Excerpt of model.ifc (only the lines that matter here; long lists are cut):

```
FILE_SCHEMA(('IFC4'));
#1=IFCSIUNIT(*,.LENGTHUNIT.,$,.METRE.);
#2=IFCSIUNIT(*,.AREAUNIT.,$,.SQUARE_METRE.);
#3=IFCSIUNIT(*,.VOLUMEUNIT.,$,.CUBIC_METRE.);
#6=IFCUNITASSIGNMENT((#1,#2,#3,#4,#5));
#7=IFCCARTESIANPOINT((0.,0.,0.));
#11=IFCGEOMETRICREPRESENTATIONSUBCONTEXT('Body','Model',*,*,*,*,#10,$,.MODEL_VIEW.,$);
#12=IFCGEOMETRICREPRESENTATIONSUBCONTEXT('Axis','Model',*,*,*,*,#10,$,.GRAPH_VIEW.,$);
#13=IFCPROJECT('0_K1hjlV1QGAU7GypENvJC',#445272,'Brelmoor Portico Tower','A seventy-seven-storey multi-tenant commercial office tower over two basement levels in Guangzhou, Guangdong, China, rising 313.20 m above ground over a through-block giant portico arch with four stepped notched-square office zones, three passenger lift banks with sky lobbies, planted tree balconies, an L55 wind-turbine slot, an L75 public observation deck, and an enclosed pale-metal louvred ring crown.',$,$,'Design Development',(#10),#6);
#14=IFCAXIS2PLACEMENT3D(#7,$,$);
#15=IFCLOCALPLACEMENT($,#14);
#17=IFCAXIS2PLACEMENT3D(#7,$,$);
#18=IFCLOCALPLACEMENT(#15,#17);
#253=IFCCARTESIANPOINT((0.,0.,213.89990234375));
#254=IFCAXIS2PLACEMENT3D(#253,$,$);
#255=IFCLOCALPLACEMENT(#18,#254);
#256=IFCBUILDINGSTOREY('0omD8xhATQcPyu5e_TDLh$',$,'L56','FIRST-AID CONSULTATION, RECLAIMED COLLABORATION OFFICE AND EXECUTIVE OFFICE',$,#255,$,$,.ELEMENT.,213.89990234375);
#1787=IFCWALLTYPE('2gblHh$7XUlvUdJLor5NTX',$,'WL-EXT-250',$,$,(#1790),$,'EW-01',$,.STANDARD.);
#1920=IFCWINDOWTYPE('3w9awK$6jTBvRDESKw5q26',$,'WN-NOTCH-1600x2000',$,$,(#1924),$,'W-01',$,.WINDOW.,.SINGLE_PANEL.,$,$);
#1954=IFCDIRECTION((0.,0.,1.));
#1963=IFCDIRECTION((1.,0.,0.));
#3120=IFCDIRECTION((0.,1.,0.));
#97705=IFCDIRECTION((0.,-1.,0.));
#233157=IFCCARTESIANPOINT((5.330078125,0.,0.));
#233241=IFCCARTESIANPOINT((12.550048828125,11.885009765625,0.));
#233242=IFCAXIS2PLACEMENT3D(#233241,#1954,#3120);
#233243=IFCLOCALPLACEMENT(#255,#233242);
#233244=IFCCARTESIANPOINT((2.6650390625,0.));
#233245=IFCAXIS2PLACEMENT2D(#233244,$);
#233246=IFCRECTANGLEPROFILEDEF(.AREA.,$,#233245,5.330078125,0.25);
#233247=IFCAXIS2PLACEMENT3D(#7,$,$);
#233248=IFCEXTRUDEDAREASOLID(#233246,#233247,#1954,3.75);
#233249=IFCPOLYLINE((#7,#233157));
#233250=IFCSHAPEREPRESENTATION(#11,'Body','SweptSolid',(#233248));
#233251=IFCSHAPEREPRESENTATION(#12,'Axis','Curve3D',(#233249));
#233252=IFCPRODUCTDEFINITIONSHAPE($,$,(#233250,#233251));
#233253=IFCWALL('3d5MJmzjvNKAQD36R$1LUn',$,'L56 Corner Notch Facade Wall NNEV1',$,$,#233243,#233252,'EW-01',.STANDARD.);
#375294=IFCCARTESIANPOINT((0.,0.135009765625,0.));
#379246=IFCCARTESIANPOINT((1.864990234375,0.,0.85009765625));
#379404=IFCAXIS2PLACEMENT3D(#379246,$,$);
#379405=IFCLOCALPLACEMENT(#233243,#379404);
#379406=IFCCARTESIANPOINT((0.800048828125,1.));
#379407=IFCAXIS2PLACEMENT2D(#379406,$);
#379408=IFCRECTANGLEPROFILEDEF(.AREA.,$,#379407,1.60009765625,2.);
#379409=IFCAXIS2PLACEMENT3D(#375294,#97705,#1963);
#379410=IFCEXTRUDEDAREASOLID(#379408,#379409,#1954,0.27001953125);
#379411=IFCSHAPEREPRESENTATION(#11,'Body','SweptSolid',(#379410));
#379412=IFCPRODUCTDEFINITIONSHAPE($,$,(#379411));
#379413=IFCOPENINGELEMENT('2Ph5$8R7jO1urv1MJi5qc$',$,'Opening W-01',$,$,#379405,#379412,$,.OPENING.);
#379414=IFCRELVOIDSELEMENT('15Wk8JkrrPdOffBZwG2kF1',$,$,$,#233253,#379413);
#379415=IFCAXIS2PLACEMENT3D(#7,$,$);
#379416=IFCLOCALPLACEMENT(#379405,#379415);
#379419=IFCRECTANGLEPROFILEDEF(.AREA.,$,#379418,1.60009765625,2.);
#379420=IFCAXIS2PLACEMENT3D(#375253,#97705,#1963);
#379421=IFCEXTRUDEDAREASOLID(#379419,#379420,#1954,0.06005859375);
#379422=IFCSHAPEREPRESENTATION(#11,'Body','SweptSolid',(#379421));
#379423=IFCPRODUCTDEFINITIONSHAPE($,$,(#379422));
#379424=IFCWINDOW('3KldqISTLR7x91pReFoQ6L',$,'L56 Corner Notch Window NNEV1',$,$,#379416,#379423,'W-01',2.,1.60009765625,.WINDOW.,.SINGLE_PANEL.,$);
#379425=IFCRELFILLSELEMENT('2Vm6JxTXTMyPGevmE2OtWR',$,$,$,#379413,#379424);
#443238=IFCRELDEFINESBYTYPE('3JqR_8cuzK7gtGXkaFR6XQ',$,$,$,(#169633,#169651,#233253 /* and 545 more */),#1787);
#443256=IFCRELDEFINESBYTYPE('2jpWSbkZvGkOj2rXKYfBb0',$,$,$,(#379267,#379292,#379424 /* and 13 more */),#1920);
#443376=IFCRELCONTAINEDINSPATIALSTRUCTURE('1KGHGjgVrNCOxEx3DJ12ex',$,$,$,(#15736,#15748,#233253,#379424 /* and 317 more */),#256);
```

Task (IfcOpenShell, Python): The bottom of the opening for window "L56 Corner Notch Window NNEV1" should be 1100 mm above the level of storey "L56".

```python
import numpy as np
import ifcopenshell
import ifcopenshell.api.geometry
import ifcopenshell.geom
import ifcopenshell.util.element
import ifcopenshell.util.placement
import ifcopenshell.util.shape
import ifcopenshell.util.unit

model = ifcopenshell.open("model.ifc")
unit_scale = ifcopenshell.util.unit.calculate_unit_scale(model)

window = model.by_id(379424)
opening = window.FillsVoids[0].RelatingOpeningElement
storey = ifcopenshell.util.element.get_container(window, ifc_class="IfcBuildingStorey")
level = ifcopenshell.util.placement.get_local_placement(storey.ObjectPlacement)[2, 3]

# The opening's origin need not be at the sill, so measure its lowest point.
shape = ifcopenshell.geom.create_shape(ifcopenshell.geom.settings(), opening)
bottom = ifcopenshell.util.shape.get_shape_bottom_elevation(shape, shape.geometry) / unit_scale
dz = level + 1.1 / unit_scale - bottom

shift = np.array([0.0, 0.0, dz])
# The window is placed relative to its opening, so it follows when the opening moves.
matrix = ifcopenshell.util.placement.get_local_placement(opening.ObjectPlacement)
matrix[:3, 3] += shift
ifcopenshell.api.geometry.edit_object_placement(
    model, product=opening, matrix=matrix, is_si=False, should_transform_children=True
)

print(f"moved by {dz * unit_scale:+.3f} m")

model.write("model_v2.ifc")
```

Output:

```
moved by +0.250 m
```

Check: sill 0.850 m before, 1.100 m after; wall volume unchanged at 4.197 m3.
